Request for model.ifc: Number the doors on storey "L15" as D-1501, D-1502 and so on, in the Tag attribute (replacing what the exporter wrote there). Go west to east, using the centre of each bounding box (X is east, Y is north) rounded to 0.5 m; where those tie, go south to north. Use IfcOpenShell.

First a look at what the model holds.

```python
import ifcopenshell
import ifcopenshell.util.element
import ifcopenshell.util.placement

model = ifcopenshell.open("model.ifc")
print(model.schema)
storey = next(s for s in model.by_type("IfcBuildingStorey") if s.Name == "L15")
doors = [e for e in ifcopenshell.util.element.get_decomposition(storey) if e.is_a("IfcDoor")]
for e in sorted(doors, key=lambda e: e.id()):
    origin = ifcopenshell.util.placement.get_local_placement(e.ObjectPlacement)[:3, 3]
    print(e.id(), e.Tag, e.Name, origin.round(2) + 0.0, sep=" | ")
```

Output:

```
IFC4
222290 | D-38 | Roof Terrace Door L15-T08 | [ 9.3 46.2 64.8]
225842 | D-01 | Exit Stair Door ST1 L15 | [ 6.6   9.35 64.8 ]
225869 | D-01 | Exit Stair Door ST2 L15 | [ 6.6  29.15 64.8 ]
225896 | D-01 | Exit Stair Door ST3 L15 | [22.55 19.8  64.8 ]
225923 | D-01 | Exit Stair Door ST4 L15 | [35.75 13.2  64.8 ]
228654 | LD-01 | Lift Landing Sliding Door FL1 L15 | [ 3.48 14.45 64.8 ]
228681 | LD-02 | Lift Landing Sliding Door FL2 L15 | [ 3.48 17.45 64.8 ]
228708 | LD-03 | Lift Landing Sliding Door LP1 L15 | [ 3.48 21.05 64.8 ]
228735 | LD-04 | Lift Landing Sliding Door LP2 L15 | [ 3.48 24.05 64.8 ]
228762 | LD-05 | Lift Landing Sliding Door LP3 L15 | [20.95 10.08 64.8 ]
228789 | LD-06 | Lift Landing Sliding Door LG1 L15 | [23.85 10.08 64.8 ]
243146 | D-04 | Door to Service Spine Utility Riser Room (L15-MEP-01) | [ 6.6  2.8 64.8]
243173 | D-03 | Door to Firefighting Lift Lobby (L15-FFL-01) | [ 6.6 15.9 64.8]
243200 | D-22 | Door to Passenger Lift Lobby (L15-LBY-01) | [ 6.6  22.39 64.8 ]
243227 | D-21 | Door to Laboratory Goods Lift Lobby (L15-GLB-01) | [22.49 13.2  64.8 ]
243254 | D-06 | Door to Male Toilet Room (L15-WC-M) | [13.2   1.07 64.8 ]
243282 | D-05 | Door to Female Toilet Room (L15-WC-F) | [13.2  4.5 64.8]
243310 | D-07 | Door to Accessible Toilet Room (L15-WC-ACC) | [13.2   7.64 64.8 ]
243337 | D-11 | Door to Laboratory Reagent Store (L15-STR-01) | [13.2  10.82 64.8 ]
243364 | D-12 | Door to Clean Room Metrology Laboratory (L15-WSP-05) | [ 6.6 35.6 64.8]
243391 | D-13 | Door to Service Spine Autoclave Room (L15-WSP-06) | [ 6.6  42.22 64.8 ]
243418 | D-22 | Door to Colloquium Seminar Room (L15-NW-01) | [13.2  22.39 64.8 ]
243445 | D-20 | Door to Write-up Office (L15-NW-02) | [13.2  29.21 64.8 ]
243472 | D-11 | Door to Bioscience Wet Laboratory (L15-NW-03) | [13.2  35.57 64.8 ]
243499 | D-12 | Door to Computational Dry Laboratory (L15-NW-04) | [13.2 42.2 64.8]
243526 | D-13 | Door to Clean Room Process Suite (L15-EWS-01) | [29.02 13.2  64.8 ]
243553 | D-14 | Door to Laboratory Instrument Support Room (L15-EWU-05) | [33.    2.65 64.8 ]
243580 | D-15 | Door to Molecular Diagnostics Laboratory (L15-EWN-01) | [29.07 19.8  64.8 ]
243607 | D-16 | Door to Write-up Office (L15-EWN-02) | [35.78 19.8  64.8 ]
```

```python
import ifcopenshell
import ifcopenshell.geom
import ifcopenshell.util.element
import ifcopenshell.util.shape

model = ifcopenshell.open("model.ifc")
settings = ifcopenshell.geom.settings()
settings.set("use-world-coords", True)


def centre(element):
    shape = ifcopenshell.geom.create_shape(settings, element)
    return ifcopenshell.util.shape.get_bbox_centroid(shape.geometry)


storey = next(s for s in model.by_type("IfcBuildingStorey") if s.Name == "L15")
doors = [e for e in ifcopenshell.util.element.get_decomposition(storey) if e.is_a("IfcDoor")]

# Insertion points can sit at a corner or the storey origin, so sort by the geometry (in metres).
centres = {e: centre(e) for e in doors}
doors.sort(key=lambda e: (round(centres[e][0] / 0.5), centres[e][1]))

for i, e in enumerate(doors, start=1):
    number = f"D-15{i:02d}"
    e.Tag = number
    print(e.id(), number)

model.write("model_rev.ifc")
```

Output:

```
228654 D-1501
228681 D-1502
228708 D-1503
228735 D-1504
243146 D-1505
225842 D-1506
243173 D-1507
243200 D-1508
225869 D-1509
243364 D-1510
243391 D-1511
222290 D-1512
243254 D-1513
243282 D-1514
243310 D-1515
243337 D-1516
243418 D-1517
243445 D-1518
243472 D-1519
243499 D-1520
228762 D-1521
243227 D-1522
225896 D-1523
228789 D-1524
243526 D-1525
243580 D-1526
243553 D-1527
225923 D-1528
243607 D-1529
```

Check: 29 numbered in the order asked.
